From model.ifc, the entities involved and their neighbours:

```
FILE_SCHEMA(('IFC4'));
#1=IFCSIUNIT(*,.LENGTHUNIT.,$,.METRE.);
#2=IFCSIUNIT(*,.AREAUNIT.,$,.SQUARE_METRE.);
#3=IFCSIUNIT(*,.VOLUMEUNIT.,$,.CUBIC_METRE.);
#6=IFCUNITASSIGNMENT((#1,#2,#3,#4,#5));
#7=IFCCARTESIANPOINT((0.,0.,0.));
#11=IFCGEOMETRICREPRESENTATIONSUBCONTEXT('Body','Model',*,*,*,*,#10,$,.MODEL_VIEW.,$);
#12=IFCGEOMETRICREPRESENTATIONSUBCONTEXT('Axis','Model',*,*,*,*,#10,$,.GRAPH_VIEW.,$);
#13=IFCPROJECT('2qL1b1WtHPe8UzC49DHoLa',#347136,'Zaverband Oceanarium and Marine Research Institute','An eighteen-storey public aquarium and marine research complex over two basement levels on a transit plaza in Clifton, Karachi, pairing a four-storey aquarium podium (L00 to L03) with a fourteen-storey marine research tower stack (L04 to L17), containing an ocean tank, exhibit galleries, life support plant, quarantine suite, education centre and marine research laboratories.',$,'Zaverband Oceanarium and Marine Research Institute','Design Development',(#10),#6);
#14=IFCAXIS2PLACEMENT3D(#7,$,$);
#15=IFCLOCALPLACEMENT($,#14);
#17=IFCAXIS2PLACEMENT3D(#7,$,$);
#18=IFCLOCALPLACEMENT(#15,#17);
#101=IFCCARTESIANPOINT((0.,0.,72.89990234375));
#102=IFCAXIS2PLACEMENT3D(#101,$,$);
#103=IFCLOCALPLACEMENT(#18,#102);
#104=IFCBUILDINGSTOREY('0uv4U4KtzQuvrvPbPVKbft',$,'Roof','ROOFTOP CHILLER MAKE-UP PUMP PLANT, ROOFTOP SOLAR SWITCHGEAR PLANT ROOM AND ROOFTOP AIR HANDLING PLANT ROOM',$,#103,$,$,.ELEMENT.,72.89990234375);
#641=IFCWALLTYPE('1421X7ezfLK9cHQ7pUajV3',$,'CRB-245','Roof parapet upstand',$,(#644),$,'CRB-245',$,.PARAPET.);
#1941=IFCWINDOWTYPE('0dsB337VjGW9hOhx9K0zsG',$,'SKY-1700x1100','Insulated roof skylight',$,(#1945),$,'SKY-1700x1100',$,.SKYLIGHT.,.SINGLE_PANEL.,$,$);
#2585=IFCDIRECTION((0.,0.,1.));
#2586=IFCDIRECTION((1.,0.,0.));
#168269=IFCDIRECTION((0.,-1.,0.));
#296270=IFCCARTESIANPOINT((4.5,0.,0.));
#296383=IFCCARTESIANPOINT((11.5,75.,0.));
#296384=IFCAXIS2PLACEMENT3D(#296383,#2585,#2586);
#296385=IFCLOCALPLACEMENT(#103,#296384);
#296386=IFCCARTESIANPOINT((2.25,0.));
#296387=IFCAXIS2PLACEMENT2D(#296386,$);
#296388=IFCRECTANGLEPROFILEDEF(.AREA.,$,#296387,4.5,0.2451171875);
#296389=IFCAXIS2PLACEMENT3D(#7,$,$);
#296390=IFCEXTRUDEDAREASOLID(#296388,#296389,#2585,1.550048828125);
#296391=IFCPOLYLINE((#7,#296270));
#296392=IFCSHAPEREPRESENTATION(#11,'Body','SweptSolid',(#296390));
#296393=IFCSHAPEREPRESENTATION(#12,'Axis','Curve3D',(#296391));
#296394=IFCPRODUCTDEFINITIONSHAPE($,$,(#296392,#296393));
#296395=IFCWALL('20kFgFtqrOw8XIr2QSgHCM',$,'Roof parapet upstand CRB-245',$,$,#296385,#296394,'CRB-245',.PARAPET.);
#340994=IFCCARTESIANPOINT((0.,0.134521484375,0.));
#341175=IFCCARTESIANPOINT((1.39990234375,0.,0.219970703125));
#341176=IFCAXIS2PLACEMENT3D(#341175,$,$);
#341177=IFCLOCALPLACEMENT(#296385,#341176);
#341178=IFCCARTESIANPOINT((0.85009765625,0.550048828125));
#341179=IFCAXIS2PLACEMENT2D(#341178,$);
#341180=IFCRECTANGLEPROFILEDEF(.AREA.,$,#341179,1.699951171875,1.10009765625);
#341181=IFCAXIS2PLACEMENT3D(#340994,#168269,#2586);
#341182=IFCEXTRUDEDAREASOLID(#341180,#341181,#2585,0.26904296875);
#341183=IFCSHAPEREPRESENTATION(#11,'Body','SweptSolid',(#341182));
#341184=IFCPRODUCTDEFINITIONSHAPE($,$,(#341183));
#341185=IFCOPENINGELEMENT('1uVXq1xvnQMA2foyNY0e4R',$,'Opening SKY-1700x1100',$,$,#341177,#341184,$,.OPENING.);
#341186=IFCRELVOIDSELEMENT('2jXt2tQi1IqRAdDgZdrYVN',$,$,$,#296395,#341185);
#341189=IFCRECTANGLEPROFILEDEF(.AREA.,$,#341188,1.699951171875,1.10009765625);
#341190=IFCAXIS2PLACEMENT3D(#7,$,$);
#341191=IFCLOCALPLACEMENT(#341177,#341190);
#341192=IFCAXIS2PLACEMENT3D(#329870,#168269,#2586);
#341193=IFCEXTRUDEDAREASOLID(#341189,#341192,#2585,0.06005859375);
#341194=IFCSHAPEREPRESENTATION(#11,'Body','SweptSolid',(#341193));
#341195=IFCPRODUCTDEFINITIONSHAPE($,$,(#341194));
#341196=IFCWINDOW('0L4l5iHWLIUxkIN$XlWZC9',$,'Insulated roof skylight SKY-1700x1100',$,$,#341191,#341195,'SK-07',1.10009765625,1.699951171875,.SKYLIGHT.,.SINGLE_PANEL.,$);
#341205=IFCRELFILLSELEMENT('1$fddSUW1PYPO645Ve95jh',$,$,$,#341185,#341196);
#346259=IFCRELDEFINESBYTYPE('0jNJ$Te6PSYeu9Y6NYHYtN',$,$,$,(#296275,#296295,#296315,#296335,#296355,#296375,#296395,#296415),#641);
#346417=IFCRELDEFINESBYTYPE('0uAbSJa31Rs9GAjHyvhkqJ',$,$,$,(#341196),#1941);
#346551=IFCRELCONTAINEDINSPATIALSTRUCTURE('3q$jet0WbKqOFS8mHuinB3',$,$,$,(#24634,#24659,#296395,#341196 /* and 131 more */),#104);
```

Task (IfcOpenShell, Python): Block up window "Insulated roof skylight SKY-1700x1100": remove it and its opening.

```python
import ifcopenshell
import ifcopenshell.api.feature
import ifcopenshell.api.root
import ifcopenshell.geom
import ifcopenshell.util.shape

model = ifcopenshell.open("model.ifc")
settings = ifcopenshell.geom.settings()


def volume(element):
    """Net volume in cubic metres, openings subtracted."""
    shape = ifcopenshell.geom.create_shape(settings, element)
    return ifcopenshell.util.shape.get_volume(shape.geometry)


window = model.by_id(341196)
opening = window.FillsVoids[0].RelatingOpeningElement
wall = opening.VoidsElements[0].RelatingBuildingElement
before = volume(wall)

ifcopenshell.api.root.remove_product(model, product=window)
ifcopenshell.api.feature.remove_feature(model, feature=opening)

after = volume(wall)

print(f"wall volume {before:.3f} -> {after:.3f} m3")

model.write("model-out.ifc")
```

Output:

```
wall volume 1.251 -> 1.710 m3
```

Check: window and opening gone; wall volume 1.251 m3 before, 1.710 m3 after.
